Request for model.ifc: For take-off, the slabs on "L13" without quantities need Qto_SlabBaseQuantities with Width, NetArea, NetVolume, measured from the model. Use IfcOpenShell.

First a look at what the model holds.

```python
import ifcopenshell
import ifcopenshell.util.element
import ifcopenshell.util.unit

model = ifcopenshell.open("model.ifc")
print(model.schema)
for unit_type in ("LENGTHUNIT", "AREAUNIT", "VOLUMEUNIT"):
    print(unit_type, ifcopenshell.util.unit.calculate_unit_scale(model, unit_type))
storey = next(s for s in model.by_type("IfcBuildingStorey") if s.Name == "L13")
slabs = [e for e in ifcopenshell.util.element.get_decomposition(storey) if e.is_a("IfcSlab")]
for e in sorted(slabs, key=lambda e: e.id()):
    print(e.id(), e.is_a(), e.Name, list(ifcopenshell.util.element.get_psets(e, qtos_only=True)), sep=" | ")
```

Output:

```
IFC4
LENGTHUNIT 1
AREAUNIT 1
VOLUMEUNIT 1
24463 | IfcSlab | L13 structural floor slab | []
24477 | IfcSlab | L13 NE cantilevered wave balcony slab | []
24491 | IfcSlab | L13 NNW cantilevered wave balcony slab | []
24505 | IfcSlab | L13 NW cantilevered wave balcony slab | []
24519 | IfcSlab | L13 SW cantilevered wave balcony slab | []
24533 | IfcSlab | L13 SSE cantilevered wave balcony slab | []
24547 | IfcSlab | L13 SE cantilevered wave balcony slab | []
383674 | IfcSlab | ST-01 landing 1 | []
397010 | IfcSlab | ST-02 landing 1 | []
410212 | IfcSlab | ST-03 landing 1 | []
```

```python
import ifcopenshell
import ifcopenshell.api.pset
import ifcopenshell.geom
import ifcopenshell.util.element
import ifcopenshell.util.shape
import ifcopenshell.util.unit

model = ifcopenshell.open("model.ifc")
unit_scale = ifcopenshell.util.unit.calculate_unit_scale(model)
area_scale = ifcopenshell.util.unit.calculate_unit_scale(model, "AREAUNIT")
volume_scale = ifcopenshell.util.unit.calculate_unit_scale(model, "VOLUMEUNIT")
settings = ifcopenshell.geom.settings()

storey = next(s for s in model.by_type("IfcBuildingStorey") if s.Name == "L13")
slabs = [e for e in ifcopenshell.util.element.get_decomposition(storey) if e.is_a("IfcSlab")]

for e in sorted(slabs, key=lambda e: e.id()):
    if ifcopenshell.util.element.get_psets(e, qtos_only=True, should_inherit=False):
        continue
    # Geometry comes back in metres, in the element's own axes.
    shape = ifcopenshell.geom.create_shape(settings, e)
    values = {
        "Width": ifcopenshell.util.shape.get_z(shape.geometry) / unit_scale,
        "NetArea": ifcopenshell.util.shape.get_footprint_area(shape.geometry) / area_scale,
        "NetVolume": ifcopenshell.util.shape.get_volume(shape.geometry) / volume_scale,
    }
    qto = ifcopenshell.api.pset.add_qto(model, product=e, name="Qto_SlabBaseQuantities")
    ifcopenshell.api.pset.edit_qto(model, qto=qto, properties=values)
    print(e.id(), {k: round(v, 3) for k, v in values.items()})

model.write("model_rev.ifc")
```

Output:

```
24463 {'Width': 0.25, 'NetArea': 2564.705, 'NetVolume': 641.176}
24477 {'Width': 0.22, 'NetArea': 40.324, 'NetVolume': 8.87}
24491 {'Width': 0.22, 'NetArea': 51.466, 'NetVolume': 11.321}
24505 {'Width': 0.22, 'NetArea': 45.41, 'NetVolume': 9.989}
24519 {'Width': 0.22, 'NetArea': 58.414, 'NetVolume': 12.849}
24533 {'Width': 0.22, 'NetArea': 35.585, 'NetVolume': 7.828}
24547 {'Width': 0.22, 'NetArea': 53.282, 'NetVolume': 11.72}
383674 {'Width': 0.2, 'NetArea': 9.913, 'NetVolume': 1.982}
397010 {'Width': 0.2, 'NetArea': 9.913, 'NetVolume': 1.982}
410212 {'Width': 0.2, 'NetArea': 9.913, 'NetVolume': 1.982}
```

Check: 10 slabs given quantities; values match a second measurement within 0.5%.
